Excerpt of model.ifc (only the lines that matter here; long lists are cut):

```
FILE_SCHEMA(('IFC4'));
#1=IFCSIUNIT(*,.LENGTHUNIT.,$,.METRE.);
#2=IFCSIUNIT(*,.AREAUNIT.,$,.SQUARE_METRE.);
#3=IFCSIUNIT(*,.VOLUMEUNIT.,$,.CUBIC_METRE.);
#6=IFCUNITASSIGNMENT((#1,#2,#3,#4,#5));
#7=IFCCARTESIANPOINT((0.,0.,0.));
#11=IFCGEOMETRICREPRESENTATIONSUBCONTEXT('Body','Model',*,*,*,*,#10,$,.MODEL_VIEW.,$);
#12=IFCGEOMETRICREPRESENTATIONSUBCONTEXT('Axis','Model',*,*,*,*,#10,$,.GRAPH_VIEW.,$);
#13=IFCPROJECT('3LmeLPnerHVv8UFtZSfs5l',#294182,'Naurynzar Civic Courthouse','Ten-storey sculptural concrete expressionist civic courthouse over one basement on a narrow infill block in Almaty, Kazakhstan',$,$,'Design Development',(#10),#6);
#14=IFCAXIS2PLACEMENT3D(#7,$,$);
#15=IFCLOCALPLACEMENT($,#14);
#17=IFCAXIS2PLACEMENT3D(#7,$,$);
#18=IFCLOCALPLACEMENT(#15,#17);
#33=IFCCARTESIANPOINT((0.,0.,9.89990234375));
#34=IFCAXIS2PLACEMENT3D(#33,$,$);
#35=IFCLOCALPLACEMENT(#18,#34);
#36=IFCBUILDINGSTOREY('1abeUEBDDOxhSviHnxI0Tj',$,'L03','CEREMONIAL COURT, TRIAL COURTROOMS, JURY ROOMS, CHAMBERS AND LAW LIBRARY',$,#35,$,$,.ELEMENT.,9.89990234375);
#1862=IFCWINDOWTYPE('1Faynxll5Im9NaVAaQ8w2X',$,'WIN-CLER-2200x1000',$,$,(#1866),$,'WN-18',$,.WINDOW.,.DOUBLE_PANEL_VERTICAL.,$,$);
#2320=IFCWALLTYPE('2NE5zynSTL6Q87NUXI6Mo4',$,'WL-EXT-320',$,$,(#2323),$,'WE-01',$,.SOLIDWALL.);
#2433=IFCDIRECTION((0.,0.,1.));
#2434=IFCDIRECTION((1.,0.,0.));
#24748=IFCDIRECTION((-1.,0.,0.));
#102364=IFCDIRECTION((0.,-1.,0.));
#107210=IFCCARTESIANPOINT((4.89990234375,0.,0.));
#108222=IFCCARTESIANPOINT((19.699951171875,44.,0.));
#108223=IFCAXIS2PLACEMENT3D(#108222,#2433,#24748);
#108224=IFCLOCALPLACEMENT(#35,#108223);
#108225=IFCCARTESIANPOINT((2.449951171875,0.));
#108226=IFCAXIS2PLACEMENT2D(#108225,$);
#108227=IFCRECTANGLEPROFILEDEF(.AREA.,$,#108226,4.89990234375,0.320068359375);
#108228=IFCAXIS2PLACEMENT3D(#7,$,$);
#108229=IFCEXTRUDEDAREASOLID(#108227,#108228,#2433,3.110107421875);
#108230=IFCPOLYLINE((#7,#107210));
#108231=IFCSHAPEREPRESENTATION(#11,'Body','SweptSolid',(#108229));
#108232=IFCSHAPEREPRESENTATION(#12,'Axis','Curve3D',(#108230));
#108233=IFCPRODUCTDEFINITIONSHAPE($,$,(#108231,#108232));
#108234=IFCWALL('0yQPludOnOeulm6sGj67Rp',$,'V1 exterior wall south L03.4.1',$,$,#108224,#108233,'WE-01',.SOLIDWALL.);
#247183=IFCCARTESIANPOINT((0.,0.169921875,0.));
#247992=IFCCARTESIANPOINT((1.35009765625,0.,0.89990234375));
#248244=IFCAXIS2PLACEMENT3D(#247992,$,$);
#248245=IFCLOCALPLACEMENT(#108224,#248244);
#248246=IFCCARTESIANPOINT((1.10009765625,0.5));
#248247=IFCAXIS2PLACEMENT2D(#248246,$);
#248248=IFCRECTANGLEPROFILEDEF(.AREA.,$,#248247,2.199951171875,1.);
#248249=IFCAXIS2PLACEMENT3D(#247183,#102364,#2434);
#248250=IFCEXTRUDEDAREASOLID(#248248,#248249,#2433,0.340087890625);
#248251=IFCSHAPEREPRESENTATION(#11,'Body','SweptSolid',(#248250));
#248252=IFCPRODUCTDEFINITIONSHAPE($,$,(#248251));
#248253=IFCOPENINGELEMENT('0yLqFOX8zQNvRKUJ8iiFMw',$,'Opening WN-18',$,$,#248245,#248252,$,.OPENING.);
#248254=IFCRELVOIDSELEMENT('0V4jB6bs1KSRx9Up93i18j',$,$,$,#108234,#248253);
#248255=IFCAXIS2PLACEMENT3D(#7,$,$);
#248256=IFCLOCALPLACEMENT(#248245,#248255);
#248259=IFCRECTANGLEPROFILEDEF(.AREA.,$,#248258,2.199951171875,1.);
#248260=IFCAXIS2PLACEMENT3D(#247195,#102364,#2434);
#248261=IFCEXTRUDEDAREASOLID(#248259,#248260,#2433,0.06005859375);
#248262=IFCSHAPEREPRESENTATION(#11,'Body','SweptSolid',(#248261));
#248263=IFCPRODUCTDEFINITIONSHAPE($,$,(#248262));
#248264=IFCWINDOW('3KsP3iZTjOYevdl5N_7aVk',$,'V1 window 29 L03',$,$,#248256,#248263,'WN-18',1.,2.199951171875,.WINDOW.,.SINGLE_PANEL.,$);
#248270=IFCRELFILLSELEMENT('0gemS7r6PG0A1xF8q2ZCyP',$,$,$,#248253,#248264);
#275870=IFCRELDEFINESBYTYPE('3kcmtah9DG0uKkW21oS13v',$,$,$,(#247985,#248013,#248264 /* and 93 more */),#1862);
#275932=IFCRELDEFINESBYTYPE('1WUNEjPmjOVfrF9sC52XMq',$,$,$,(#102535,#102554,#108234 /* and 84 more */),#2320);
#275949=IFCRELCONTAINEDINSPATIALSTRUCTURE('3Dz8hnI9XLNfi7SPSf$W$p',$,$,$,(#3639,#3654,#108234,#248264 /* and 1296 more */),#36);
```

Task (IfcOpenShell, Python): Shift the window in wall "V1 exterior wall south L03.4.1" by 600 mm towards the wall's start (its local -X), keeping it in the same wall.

```python
import ifcopenshell
import ifcopenshell.api.geometry
import ifcopenshell.util.placement

model = ifcopenshell.open("model.ifc")

window = model.by_guid("3KsP3iZTjOYevdl5N_7aVk")
opening = window.FillsVoids[0].RelatingOpeningElement
wall = opening.VoidsElements[0].RelatingBuildingElement

wall_matrix = ifcopenshell.util.placement.get_local_placement(wall.ObjectPlacement)
shift = wall_matrix[:3, 0] * -0.6
before = ifcopenshell.util.placement.get_local_placement(window.ObjectPlacement)[:3, 3].copy()

# The window is placed relative to its opening, so it follows when the opening moves.
matrix = ifcopenshell.util.placement.get_local_placement(opening.ObjectPlacement)
matrix[:3, 3] += shift
ifcopenshell.api.geometry.edit_object_placement(
    model, product=opening, matrix=matrix, is_si=False, should_transform_children=True
)

after = ifcopenshell.util.placement.get_local_placement(window.ObjectPlacement)[:3, 3]
print("window moved by", (after - before).round(3) + 0.0)

model.write("model_rev.ifc")
```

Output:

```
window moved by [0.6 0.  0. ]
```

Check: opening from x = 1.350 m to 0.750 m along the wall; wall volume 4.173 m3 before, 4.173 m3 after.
